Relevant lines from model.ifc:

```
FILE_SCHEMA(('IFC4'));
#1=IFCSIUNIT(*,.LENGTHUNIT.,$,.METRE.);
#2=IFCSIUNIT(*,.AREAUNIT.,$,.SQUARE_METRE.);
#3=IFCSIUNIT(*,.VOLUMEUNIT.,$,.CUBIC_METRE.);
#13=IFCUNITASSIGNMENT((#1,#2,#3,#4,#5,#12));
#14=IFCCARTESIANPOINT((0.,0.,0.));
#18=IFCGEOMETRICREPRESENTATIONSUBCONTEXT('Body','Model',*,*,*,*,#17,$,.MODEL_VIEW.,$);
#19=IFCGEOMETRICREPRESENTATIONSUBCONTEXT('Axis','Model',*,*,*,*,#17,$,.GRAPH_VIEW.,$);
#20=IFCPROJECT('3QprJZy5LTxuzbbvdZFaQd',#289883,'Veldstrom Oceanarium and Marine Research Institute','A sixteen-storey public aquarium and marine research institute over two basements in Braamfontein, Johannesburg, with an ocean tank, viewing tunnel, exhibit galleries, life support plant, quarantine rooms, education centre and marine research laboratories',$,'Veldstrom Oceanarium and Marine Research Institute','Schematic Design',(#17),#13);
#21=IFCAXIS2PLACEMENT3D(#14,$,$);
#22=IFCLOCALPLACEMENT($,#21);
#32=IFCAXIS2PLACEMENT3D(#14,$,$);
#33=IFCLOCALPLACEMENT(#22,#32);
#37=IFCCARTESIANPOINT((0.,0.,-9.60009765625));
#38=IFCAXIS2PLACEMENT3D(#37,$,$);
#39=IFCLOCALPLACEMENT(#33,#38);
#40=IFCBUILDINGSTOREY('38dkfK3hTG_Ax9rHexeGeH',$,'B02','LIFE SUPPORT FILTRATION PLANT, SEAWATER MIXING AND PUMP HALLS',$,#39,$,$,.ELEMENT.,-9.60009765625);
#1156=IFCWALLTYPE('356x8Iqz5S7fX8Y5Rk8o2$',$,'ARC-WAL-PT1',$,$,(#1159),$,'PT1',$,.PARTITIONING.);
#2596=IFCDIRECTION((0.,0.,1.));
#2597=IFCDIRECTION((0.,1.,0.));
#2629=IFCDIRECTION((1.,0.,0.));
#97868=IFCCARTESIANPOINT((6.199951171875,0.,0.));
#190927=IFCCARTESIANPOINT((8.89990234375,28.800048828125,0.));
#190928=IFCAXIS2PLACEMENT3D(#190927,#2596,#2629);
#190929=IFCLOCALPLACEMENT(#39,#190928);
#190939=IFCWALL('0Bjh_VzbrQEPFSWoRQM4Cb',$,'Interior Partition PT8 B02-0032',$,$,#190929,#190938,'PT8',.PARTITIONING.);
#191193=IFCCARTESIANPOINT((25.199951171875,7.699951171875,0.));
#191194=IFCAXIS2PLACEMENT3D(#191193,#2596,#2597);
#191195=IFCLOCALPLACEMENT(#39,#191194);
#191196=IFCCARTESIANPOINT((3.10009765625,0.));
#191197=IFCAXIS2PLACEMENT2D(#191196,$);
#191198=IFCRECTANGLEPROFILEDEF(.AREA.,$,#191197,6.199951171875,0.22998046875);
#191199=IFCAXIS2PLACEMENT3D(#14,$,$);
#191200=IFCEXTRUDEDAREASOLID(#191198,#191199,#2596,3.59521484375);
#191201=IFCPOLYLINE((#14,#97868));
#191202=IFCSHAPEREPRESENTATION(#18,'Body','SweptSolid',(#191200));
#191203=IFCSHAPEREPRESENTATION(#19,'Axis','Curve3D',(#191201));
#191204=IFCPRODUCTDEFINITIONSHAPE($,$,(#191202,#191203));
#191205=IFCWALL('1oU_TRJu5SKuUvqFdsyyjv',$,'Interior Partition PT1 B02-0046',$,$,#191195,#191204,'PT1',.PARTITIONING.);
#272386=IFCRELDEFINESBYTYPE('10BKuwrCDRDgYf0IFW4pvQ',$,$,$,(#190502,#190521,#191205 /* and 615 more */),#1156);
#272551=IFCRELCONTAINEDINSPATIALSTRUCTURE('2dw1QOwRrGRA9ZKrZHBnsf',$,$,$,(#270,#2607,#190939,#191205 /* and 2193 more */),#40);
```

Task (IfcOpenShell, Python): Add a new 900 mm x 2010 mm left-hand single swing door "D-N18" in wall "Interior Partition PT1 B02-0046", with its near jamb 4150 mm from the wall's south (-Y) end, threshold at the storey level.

```python
import numpy as np
import ifcopenshell
import ifcopenshell.api.feature
import ifcopenshell.api.geometry
import ifcopenshell.api.root
import ifcopenshell.api.spatial
import ifcopenshell.geom
import ifcopenshell.util.element
import ifcopenshell.util.placement
import ifcopenshell.util.representation
import ifcopenshell.util.shape
import ifcopenshell.util.unit

model = ifcopenshell.open("model.ifc")
unit_scale = ifcopenshell.util.unit.calculate_unit_scale(model)
settings = ifcopenshell.geom.settings()


def volume(element):
    """Net volume in cubic metres, openings subtracted."""
    shape = ifcopenshell.geom.create_shape(settings, element)
    return ifcopenshell.util.shape.get_volume(shape.geometry)


wall = model.by_guid("1oU_TRJu5SKuUvqFdsyyjv")
storey = ifcopenshell.util.element.get_container(wall, ifc_class="IfcBuildingStorey")
context = ifcopenshell.util.representation.get_context(model, "Model", "Body", "MODEL_VIEW")
before = volume(wall)

width, height, from_end, sill = 0.9, 2.01, 4.15, 0.0  # metres

# The wall runs along its own X axis, and the end named is its -X end.
wall_shape = ifcopenshell.geom.create_shape(settings, wall)
x, y, z = ifcopenshell.util.shape.get_vertices(wall_shape.geometry).T
start = x.min() + from_end
face, thickness = float(y.min()), float(y.max() - y.min())
wall_matrix = ifcopenshell.util.placement.get_local_placement(wall.ObjectPlacement)
level = ifcopenshell.util.placement.get_local_placement(storey.ObjectPlacement)[2, 3]


def in_wall(x, y):
    """Placement at x, y metres in the wall's axes, at sill height."""
    matrix = wall_matrix.copy()
    matrix[:, 3] = wall_matrix @ np.array([x / unit_scale, y / unit_scale, 0.0, 1.0])
    matrix[2, 3] = level + sill / unit_scale
    return matrix


# Opening: a box that overshoots both wall faces by 50 mm.
opening = ifcopenshell.api.root.create_entity(model, ifc_class="IfcOpeningElement", predefined_type="OPENING")
box = ifcopenshell.api.geometry.add_wall_representation(
    model, context=context, length=width, height=height, thickness=thickness + 0.1
)
ifcopenshell.api.geometry.assign_representation(model, product=opening, representation=box)
ifcopenshell.api.geometry.edit_object_placement(model, product=opening, matrix=in_wall(start, face - 0.05), is_si=False)
ifcopenshell.api.feature.add_feature(model, feature=opening, element=wall)

door = ifcopenshell.api.root.create_entity(model, ifc_class="IfcDoor", name="D-N18", predefined_type="DOOR")
door.OverallWidth, door.OverallHeight = width / unit_scale, height / unit_scale
door.OperationType = "SINGLE_SWING_LEFT"
body = ifcopenshell.api.geometry.add_door_representation(
    model,
    context=context,
    overall_width=door.OverallWidth,
    overall_height=door.OverallHeight,
    operation_type="SINGLE_SWING_LEFT",
    lining_properties={"LiningDepth": thickness / unit_scale, "ThresholdDepth": thickness / unit_scale},
)
ifcopenshell.api.geometry.assign_representation(model, product=door, representation=body)
ifcopenshell.api.spatial.assign_container(model, products=[door], relating_structure=storey)
ifcopenshell.api.feature.add_filling(model, opening=opening, element=door)

# The lining spans the wall, so the door starts at the wall face.
ifcopenshell.api.geometry.edit_object_placement(model, product=door, matrix=in_wall(start, face), is_si=False)

after = volume(wall)

print(f"wall volume {before:.3f} -> {after:.3f} m3")

model.write("model_edited.ifc")
```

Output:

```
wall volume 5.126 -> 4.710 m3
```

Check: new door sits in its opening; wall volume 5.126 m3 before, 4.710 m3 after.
